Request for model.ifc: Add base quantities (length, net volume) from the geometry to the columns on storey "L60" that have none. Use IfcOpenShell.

First a look at what the model holds.

```python
import ifcopenshell
import ifcopenshell.util.element
import ifcopenshell.util.unit

model = ifcopenshell.open("model.ifc")
print(model.schema)
for unit_type in ("LENGTHUNIT", "AREAUNIT", "VOLUMEUNIT"):
    print(unit_type, ifcopenshell.util.unit.calculate_unit_scale(model, unit_type))
storey = next(s for s in model.by_type("IfcBuildingStorey") if s.Name == "L60")
columns = [e for e in ifcopenshell.util.element.get_decomposition(storey) if e.is_a("IfcColumn")]
for e in sorted(columns, key=lambda e: e.id()):
    print(e.id(), e.is_a(), e.Name, list(ifcopenshell.util.element.get_psets(e, qtos_only=True)), sep=" | ")
```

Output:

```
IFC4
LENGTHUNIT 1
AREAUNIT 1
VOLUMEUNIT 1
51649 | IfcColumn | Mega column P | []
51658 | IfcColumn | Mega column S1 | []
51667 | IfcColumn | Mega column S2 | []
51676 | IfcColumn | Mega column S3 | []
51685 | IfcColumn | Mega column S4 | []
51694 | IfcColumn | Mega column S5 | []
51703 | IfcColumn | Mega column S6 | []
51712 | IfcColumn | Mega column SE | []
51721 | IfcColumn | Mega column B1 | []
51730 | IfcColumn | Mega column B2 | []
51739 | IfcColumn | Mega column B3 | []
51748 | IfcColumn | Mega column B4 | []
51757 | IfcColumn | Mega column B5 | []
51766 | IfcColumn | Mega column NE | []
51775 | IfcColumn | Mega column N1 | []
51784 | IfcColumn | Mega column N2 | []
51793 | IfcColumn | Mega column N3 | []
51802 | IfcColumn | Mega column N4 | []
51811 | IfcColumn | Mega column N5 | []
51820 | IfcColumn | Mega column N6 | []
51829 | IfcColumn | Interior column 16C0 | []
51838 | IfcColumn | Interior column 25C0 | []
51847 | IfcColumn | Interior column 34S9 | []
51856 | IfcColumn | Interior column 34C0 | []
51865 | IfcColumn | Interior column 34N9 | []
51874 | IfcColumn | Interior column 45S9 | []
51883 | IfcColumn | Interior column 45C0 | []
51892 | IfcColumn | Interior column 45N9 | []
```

```python
import ifcopenshell
import ifcopenshell.api.pset
import ifcopenshell.geom
import ifcopenshell.util.element
import ifcopenshell.util.shape
import ifcopenshell.util.unit

model = ifcopenshell.open("model.ifc")
unit_scale = ifcopenshell.util.unit.calculate_unit_scale(model)
volume_scale = ifcopenshell.util.unit.calculate_unit_scale(model, "VOLUMEUNIT")
settings = ifcopenshell.geom.settings()

storey = next(s for s in model.by_type("IfcBuildingStorey") if s.Name == "L60")
columns = [e for e in ifcopenshell.util.element.get_decomposition(storey) if e.is_a("IfcColumn")]

for e in sorted(columns, key=lambda e: e.id()):
    if ifcopenshell.util.element.get_psets(e, qtos_only=True, should_inherit=False):
        continue
    # Geometry comes back in metres, in the element's own axes.
    shape = ifcopenshell.geom.create_shape(settings, e)
    values = {
        "Length": ifcopenshell.util.shape.get_z(shape.geometry) / unit_scale,
        "NetVolume": ifcopenshell.util.shape.get_volume(shape.geometry) / volume_scale,
    }
    qto = ifcopenshell.api.pset.add_qto(model, product=e, name="Qto_ColumnBaseQuantities")
    ifcopenshell.api.pset.edit_qto(model, qto=qto, properties=values)
    print(e.id(), {k: round(v, 3) for k, v in values.items()})

model.write("model-out.ifc")
```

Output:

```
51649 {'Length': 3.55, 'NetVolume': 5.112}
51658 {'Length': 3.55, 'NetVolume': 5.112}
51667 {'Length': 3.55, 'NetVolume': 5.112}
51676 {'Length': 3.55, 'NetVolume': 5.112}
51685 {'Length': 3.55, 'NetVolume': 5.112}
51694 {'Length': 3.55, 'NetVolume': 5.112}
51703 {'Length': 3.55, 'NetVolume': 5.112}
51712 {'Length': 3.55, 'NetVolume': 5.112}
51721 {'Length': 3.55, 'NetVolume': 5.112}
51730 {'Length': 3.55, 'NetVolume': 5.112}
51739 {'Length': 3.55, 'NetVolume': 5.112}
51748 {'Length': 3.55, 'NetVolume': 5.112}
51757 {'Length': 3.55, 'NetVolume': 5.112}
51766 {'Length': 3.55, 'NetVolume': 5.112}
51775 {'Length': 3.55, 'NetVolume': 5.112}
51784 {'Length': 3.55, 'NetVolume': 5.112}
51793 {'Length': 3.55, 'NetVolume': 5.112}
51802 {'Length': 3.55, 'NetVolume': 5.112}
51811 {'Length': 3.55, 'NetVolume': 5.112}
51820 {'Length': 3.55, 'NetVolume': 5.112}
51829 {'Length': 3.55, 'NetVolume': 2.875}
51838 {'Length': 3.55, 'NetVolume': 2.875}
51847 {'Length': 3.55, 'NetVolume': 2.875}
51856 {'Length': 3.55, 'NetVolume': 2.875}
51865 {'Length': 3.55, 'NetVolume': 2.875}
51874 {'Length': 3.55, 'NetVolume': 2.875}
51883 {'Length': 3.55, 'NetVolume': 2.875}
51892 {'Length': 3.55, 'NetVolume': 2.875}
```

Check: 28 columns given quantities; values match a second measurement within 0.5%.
